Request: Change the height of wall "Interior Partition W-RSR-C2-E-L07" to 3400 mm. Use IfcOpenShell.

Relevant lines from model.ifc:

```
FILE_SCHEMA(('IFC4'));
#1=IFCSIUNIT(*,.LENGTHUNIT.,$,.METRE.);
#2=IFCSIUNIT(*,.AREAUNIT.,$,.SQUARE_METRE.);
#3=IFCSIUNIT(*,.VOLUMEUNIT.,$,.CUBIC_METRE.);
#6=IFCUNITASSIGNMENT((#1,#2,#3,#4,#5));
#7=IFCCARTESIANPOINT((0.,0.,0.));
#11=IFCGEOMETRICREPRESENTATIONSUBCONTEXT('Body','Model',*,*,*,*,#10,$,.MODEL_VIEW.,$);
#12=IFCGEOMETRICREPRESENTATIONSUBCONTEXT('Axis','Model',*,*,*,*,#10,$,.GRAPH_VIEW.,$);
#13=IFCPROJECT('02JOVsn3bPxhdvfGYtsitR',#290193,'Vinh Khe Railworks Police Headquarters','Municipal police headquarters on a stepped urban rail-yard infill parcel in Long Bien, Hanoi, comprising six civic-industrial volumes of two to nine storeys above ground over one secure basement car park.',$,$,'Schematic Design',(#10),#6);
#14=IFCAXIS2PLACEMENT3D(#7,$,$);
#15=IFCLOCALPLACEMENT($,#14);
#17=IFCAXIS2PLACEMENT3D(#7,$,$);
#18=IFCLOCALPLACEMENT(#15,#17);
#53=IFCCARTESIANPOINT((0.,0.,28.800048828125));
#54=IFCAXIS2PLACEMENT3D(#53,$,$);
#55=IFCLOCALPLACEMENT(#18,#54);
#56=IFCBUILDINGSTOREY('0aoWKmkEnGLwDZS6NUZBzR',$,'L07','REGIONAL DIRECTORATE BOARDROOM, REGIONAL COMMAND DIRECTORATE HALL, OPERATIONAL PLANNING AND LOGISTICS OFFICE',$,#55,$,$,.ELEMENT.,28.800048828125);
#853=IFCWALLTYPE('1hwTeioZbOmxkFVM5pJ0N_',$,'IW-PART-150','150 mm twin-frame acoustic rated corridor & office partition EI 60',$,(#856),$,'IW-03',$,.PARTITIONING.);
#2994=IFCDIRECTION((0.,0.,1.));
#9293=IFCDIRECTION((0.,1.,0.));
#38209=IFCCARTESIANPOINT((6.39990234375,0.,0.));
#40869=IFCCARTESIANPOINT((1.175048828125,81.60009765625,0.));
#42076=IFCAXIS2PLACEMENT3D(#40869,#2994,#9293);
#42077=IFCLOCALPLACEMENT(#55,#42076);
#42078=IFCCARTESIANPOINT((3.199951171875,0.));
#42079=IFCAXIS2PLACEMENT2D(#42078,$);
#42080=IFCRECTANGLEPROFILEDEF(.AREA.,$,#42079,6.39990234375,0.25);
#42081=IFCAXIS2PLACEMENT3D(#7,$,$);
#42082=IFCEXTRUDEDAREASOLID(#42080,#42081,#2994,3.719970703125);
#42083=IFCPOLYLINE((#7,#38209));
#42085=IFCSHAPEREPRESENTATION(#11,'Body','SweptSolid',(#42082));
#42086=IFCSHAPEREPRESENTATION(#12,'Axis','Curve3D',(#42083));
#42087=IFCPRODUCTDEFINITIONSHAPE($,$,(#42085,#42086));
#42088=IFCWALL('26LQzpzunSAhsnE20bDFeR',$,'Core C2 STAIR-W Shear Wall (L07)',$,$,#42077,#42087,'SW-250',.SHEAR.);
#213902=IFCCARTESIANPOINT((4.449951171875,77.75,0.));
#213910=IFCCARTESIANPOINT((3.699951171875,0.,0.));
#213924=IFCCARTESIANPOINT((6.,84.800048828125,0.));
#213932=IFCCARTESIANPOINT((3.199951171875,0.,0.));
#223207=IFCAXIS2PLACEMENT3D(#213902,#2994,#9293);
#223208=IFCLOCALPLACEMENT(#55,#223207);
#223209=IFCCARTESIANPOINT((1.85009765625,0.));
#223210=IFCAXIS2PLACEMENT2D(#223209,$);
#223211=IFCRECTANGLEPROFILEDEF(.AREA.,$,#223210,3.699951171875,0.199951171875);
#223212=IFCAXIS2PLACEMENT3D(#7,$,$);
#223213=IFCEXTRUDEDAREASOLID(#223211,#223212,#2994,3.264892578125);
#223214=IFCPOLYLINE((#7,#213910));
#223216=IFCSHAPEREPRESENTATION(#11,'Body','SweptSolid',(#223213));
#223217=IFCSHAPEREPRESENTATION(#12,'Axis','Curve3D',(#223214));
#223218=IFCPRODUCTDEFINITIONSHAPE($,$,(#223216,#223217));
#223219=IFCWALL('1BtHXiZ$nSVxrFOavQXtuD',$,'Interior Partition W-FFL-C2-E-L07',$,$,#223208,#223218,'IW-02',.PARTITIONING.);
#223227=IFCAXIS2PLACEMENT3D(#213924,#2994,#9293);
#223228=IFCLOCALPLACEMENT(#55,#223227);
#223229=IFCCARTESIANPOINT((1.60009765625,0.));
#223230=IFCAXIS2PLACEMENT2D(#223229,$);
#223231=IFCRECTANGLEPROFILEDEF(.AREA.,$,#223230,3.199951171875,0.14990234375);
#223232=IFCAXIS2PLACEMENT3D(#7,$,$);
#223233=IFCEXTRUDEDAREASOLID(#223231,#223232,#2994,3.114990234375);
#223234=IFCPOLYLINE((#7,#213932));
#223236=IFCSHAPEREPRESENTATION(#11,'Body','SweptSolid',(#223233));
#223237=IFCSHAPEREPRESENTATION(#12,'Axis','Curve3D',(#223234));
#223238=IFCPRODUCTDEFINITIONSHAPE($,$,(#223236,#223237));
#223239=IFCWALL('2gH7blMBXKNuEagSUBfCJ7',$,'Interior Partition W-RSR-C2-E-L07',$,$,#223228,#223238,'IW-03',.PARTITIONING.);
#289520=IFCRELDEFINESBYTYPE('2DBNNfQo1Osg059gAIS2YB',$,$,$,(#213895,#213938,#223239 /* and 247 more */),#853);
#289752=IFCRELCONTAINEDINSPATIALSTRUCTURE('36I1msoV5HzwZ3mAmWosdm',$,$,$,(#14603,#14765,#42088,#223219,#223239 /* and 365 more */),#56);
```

```python
import ifcopenshell
import ifcopenshell.geom
import ifcopenshell.util.representation
import ifcopenshell.util.shape
import ifcopenshell.util.unit

model = ifcopenshell.open("model.ifc")
unit_scale = ifcopenshell.util.unit.calculate_unit_scale(model)
settings = ifcopenshell.geom.settings()


def volume(element):
    """Net volume in cubic metres, openings subtracted."""
    shape = ifcopenshell.geom.create_shape(settings, element)
    return ifcopenshell.util.shape.get_volume(shape.geometry)


wall = model.by_guid("2gH7blMBXKNuEagSUBfCJ7")
before = volume(wall)

body = ifcopenshell.util.representation.get_representation(wall, "Model", "Body")
solid = body.Items[0]
old_height = solid.Depth
solid.Depth = 3.4 / unit_scale
after = volume(wall)

print(f"height {old_height:g} -> {solid.Depth:g}, volume {before:.3f} -> {after:.3f} m3")

model.write("model_updated.ifc")
```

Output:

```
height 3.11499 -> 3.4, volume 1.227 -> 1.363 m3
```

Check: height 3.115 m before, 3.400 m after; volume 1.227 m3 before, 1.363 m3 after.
